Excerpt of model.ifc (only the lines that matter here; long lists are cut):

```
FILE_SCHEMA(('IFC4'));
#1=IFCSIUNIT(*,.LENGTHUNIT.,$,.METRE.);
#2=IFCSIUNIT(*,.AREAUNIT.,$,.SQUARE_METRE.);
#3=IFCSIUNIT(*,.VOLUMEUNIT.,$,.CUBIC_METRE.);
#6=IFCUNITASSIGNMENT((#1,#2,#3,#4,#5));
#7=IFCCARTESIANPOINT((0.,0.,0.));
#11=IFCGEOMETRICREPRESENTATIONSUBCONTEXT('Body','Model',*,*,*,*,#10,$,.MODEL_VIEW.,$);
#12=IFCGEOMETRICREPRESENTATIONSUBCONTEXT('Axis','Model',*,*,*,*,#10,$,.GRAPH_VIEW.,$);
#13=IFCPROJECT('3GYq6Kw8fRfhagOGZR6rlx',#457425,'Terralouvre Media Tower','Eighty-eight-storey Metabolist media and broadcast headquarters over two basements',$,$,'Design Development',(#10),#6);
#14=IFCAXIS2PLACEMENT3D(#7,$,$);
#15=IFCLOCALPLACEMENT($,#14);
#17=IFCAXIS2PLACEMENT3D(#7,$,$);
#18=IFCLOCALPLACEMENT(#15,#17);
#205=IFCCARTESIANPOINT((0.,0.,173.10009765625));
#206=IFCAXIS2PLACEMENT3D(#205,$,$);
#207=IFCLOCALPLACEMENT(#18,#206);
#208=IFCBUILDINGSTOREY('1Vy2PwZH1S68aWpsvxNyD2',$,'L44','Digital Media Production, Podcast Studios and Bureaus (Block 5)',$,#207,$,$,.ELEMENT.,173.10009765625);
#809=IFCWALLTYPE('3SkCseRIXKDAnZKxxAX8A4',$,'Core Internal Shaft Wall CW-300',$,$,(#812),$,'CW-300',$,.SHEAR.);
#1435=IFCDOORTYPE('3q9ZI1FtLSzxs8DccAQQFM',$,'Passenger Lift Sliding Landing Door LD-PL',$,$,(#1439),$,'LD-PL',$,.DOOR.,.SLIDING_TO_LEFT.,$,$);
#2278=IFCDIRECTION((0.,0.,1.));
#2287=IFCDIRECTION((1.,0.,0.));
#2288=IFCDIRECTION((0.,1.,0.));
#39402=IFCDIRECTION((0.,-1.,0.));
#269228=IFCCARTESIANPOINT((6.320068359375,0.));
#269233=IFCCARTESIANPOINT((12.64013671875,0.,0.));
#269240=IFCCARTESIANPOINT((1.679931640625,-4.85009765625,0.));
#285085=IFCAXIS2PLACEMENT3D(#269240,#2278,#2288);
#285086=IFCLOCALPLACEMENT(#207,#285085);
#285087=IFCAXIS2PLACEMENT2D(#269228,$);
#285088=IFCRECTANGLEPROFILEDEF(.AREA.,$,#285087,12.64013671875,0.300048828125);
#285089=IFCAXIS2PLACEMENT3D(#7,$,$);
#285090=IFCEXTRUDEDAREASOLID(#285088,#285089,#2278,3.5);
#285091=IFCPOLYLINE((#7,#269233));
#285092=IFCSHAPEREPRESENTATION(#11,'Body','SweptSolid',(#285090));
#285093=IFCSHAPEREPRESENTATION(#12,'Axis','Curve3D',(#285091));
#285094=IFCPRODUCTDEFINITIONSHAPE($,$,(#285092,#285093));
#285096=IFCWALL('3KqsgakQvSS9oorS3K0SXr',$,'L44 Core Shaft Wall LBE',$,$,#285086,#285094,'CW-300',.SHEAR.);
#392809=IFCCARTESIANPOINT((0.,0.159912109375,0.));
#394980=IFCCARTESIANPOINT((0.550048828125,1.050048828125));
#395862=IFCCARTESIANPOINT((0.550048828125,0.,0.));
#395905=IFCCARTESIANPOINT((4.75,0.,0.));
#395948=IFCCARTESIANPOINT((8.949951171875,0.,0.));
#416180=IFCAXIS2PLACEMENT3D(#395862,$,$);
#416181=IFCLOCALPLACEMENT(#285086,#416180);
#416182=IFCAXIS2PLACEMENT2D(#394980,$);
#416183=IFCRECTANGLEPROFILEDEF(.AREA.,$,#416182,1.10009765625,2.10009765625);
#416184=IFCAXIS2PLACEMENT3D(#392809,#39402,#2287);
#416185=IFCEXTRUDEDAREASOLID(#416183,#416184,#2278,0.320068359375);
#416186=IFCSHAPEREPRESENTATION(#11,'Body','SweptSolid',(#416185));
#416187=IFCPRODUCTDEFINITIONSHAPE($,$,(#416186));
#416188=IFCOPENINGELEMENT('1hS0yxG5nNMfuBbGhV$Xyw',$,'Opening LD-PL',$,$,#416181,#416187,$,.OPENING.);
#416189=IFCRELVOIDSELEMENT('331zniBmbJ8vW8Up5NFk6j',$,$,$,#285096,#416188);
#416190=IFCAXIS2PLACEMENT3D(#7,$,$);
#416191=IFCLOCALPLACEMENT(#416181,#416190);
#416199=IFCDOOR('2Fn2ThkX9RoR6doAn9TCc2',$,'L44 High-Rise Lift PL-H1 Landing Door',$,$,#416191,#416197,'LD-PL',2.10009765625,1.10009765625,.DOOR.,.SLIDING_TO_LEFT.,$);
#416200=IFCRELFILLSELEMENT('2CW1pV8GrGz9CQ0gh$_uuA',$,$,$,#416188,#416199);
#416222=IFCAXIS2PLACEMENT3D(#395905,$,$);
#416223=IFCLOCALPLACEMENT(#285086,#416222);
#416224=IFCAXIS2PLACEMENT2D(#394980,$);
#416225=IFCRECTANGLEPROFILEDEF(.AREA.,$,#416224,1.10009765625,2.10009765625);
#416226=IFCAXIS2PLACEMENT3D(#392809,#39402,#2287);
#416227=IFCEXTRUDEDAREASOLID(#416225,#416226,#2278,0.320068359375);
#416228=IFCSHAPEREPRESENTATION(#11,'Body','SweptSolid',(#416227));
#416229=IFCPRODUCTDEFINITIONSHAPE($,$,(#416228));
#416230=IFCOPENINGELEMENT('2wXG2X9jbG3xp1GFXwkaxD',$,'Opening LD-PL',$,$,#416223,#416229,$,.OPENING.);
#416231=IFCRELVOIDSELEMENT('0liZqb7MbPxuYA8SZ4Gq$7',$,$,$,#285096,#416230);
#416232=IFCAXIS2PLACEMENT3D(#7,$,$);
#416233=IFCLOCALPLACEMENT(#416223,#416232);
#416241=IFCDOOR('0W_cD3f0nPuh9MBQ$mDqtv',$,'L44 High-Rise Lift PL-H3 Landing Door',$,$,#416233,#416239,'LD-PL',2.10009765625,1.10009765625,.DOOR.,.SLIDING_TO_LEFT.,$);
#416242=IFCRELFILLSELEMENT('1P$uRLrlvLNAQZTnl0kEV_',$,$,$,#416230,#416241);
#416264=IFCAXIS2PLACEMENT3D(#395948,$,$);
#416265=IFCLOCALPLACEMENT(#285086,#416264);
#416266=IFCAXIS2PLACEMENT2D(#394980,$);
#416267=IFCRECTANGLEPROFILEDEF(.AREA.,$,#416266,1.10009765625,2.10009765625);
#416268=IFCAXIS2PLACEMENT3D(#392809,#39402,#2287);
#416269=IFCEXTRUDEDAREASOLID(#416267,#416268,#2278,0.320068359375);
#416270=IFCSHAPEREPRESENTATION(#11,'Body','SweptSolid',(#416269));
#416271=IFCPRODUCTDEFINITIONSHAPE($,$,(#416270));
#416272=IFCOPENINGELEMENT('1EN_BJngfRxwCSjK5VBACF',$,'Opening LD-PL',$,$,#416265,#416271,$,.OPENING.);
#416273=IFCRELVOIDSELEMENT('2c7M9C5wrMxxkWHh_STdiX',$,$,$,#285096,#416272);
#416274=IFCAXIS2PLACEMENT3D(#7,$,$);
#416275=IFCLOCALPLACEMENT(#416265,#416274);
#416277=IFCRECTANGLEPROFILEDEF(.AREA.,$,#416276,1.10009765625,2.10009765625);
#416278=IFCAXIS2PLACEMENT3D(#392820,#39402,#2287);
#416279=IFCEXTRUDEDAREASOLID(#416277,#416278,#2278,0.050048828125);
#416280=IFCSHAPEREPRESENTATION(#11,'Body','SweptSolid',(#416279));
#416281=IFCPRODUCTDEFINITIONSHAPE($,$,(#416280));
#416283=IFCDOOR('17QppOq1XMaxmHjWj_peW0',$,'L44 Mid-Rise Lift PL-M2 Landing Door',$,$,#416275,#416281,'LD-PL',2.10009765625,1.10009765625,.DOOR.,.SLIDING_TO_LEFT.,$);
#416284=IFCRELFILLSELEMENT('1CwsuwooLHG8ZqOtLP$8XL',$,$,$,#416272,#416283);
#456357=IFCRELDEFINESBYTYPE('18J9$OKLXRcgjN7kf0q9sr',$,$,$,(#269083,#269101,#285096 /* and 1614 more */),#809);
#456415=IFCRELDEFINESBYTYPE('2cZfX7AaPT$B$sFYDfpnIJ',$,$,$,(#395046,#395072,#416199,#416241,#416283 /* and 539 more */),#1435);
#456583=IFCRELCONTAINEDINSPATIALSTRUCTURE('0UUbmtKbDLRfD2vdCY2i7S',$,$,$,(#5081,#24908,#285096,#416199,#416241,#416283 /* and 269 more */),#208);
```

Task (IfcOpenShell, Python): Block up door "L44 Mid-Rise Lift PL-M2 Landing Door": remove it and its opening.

```python
import ifcopenshell
import ifcopenshell.api.feature
import ifcopenshell.api.root
import ifcopenshell.geom
import ifcopenshell.util.shape

model = ifcopenshell.open("model.ifc")
settings = ifcopenshell.geom.settings()


def volume(element):
    """Net volume in cubic metres, openings subtracted."""
    shape = ifcopenshell.geom.create_shape(settings, element)
    return ifcopenshell.util.shape.get_volume(shape.geometry)


door = model.by_guid("17QppOq1XMaxmHjWj_peW0")
opening = door.FillsVoids[0].RelatingOpeningElement
wall = opening.VoidsElements[0].RelatingBuildingElement
before = volume(wall)

ifcopenshell.api.root.remove_product(model, product=door)
ifcopenshell.api.feature.remove_feature(model, feature=opening)

after = volume(wall)

print(f"wall volume {before:.3f} -> {after:.3f} m3")

model.write("model_updated.ifc")
```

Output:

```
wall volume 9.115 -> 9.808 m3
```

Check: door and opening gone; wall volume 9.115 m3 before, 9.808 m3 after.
